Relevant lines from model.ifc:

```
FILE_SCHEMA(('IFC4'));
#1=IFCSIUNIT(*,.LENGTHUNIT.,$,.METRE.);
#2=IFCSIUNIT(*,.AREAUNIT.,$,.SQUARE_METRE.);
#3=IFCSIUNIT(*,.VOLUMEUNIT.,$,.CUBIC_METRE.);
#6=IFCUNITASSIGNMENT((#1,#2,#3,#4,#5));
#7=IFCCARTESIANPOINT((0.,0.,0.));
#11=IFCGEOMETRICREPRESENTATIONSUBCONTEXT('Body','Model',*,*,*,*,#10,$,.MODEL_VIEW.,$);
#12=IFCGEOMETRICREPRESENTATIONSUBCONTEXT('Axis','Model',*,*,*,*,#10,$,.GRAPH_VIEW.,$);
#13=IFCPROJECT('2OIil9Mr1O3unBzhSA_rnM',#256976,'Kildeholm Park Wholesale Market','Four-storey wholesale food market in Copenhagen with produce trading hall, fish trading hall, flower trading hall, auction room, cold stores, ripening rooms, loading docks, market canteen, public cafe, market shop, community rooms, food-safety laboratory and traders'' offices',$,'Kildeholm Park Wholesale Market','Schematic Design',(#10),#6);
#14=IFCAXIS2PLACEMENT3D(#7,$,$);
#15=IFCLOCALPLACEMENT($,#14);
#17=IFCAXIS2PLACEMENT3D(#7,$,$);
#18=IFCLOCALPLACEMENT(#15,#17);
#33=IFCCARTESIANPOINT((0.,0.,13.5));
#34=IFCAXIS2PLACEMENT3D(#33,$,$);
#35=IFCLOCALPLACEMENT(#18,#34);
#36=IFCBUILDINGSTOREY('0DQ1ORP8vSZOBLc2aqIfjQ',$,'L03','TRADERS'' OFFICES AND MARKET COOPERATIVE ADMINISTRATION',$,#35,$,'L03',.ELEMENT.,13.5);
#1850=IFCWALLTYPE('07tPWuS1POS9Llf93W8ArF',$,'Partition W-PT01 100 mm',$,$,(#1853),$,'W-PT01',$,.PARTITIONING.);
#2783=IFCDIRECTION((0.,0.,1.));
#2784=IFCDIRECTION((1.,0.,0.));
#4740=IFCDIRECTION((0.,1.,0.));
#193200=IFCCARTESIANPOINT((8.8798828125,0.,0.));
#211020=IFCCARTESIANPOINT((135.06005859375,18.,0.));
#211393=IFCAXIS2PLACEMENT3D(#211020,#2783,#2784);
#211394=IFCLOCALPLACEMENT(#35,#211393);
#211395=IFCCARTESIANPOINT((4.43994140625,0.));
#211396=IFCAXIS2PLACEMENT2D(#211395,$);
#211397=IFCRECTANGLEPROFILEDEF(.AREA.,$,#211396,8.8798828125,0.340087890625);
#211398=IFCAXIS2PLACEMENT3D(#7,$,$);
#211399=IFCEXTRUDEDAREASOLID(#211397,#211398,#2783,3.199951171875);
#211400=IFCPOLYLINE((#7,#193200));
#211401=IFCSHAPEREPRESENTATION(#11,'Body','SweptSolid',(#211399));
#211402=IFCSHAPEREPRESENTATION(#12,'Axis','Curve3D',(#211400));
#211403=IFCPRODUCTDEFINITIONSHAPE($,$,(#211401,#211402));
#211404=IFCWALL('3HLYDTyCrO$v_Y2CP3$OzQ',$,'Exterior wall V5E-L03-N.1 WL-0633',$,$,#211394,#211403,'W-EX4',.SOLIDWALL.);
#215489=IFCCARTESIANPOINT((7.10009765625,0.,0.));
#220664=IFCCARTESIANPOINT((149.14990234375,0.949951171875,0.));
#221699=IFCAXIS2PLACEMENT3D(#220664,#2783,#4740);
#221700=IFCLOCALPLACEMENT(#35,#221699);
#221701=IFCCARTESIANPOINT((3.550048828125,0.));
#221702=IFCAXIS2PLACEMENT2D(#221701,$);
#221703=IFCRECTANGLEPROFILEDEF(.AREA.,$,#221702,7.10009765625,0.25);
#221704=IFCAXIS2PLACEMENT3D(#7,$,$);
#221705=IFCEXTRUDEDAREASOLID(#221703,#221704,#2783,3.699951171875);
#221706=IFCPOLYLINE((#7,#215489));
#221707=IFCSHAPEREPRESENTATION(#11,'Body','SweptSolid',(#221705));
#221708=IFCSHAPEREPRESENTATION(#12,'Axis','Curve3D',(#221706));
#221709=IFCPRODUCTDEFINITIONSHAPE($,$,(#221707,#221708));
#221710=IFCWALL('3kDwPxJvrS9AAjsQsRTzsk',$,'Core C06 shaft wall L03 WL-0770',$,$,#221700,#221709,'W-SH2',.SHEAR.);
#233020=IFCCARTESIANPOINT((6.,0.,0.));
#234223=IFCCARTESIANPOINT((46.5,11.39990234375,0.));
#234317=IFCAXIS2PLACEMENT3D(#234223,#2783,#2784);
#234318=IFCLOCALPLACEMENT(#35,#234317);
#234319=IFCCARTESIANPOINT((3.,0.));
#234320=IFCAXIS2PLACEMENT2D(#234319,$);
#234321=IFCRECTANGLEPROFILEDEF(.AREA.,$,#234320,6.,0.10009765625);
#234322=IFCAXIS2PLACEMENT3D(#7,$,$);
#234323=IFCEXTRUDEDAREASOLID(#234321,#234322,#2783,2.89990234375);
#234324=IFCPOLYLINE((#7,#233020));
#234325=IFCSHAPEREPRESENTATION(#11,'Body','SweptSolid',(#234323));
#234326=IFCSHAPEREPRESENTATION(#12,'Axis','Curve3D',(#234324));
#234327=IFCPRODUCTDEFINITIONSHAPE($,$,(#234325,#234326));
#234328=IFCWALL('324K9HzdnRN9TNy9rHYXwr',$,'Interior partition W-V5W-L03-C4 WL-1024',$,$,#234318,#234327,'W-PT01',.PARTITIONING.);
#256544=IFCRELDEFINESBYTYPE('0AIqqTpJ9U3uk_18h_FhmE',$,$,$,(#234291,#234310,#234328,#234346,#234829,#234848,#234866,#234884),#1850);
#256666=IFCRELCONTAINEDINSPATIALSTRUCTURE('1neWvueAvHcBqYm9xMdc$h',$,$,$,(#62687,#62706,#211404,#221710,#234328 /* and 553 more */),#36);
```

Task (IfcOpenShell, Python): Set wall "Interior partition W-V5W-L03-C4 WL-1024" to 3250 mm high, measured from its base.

```python
import ifcopenshell
import ifcopenshell.geom
import ifcopenshell.util.representation
import ifcopenshell.util.shape
import ifcopenshell.util.unit

model = ifcopenshell.open("model.ifc")
unit_scale = ifcopenshell.util.unit.calculate_unit_scale(model)
settings = ifcopenshell.geom.settings()


def volume(element):
    """Net volume in cubic metres, openings subtracted."""
    shape = ifcopenshell.geom.create_shape(settings, element)
    return ifcopenshell.util.shape.get_volume(shape.geometry)


wall = model.by_guid("324K9HzdnRN9TNy9rHYXwr")
before = volume(wall)

body = ifcopenshell.util.representation.get_representation(wall, "Model", "Body")
solid = body.Items[0]
old_height = solid.Depth
solid.Depth = 3.25 / unit_scale
after = volume(wall)

print(f"height {old_height:g} -> {solid.Depth:g}, volume {before:.3f} -> {after:.3f} m3")

model.write("model_updated.ifc")
```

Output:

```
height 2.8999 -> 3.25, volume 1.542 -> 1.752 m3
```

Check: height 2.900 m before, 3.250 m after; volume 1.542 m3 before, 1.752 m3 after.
